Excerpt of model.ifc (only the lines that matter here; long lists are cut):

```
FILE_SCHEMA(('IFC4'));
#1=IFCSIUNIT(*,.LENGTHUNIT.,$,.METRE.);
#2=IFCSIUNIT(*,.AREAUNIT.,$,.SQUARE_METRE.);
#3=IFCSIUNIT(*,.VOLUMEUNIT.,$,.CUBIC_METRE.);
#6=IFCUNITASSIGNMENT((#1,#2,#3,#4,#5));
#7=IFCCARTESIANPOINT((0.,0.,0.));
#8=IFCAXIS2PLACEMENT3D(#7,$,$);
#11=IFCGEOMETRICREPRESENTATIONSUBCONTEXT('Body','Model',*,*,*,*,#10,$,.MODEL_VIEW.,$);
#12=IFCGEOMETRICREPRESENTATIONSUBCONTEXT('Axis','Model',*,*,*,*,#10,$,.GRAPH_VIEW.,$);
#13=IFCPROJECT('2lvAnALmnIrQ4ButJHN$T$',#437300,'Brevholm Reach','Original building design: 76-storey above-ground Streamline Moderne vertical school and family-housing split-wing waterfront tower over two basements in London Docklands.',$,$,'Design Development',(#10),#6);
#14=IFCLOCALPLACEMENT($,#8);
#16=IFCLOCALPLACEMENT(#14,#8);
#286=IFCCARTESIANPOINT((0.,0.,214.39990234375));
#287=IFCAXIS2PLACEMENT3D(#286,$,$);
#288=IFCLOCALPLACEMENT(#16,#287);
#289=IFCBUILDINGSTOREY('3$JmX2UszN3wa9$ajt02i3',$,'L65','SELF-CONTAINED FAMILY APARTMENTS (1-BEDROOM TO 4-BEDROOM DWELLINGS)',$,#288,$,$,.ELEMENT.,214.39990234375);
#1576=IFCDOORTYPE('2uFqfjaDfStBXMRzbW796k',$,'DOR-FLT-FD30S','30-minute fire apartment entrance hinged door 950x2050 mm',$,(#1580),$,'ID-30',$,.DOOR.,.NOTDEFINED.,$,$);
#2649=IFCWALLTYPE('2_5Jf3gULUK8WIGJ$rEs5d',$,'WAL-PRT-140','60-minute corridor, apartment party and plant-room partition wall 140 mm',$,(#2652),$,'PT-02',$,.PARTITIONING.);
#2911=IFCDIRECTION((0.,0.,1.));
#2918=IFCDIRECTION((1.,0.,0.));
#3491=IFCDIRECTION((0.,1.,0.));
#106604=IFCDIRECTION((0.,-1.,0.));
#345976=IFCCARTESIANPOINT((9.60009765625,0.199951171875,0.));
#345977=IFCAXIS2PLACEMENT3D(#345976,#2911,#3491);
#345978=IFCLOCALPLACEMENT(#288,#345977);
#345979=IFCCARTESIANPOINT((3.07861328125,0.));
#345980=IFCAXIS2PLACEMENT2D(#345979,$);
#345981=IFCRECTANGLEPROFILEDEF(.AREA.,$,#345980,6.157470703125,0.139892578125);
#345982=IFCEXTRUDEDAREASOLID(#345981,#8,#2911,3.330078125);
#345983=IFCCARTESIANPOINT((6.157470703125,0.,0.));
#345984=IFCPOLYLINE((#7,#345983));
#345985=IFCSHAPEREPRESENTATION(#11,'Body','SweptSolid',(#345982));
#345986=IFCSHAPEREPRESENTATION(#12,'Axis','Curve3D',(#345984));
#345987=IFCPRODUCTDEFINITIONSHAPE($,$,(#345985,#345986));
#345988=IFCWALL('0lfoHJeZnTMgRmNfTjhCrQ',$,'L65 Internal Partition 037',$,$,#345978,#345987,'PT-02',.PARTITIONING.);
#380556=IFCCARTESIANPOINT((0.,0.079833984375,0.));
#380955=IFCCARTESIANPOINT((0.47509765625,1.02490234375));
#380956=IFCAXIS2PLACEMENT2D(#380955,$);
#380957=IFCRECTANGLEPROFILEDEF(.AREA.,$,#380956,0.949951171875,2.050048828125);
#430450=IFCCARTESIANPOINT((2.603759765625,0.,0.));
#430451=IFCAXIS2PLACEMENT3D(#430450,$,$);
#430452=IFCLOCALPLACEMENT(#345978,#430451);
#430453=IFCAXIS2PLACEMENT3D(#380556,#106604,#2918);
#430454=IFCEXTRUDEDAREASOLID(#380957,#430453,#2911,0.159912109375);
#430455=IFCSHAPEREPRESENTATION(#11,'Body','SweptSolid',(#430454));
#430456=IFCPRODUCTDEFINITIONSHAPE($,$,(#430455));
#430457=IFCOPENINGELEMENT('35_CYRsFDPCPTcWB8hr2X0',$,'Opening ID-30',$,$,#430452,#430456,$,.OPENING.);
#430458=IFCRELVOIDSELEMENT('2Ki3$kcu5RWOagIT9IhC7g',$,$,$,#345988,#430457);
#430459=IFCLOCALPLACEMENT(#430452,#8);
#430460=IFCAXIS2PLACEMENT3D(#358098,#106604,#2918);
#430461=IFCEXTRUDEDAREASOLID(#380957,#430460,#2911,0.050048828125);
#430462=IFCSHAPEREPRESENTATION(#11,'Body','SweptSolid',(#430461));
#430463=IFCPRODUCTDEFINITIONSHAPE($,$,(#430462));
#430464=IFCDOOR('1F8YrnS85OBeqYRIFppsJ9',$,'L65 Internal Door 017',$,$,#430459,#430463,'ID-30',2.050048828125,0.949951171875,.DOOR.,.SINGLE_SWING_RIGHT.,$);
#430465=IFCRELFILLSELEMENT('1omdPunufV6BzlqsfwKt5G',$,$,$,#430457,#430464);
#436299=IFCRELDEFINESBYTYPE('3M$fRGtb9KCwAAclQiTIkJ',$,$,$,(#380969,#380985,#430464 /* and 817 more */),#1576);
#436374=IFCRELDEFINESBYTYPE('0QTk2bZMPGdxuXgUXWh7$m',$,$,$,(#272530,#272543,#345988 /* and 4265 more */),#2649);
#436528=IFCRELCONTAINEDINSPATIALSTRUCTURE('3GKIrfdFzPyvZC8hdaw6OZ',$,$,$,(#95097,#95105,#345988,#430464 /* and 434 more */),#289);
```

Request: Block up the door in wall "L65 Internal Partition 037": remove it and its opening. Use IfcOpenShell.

```python
import ifcopenshell
import ifcopenshell.api.feature
import ifcopenshell.api.root
import ifcopenshell.geom
import ifcopenshell.util.shape

model = ifcopenshell.open("model.ifc")
settings = ifcopenshell.geom.settings()


def volume(element):
    """Net volume in cubic metres, openings subtracted."""
    shape = ifcopenshell.geom.create_shape(settings, element)
    return ifcopenshell.util.shape.get_volume(shape.geometry)


door = model.by_guid("1F8YrnS85OBeqYRIFppsJ9")
opening = door.FillsVoids[0].RelatingOpeningElement
wall = opening.VoidsElements[0].RelatingBuildingElement
before = volume(wall)

ifcopenshell.api.root.remove_product(model, product=door)
ifcopenshell.api.feature.remove_feature(model, feature=opening)

after = volume(wall)

print(f"wall volume {before:.3f} -> {after:.3f} m3")

model.write("model_edited.ifc")
```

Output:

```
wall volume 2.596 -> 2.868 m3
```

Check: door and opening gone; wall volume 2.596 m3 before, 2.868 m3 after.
